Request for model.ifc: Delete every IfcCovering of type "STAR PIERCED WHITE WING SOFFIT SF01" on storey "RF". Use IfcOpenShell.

First a look at what the model holds.

```python
import ifcopenshell
import ifcopenshell.util.element

model = ifcopenshell.open("model.ifc")
print(model.schema)
storey = next(s for s in model.by_type("IfcBuildingStorey") if s.Name == "RF")
coverings = [e for e in ifcopenshell.util.element.get_decomposition(storey) if e.is_a("IfcCovering")]
seen = {}
for e in coverings:
    element_type = ifcopenshell.util.element.get_type(e)
    name = element_type.Name if element_type not in (None, e) else None
    seen[name] = seen.get(name, 0) + 1
for name, count in sorted(seen.items(), key=str):
    print(count, "x", name)
```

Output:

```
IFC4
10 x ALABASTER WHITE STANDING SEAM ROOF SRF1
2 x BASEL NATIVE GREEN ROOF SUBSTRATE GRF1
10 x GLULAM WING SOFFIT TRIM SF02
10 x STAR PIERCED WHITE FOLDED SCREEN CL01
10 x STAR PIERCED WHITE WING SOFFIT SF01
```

```python
import ifcopenshell
import ifcopenshell.api.root
import ifcopenshell.util.element

model = ifcopenshell.open("model.ifc")

storey = next(s for s in model.by_type("IfcBuildingStorey") if s.Name == "RF")
coverings = [e for e in ifcopenshell.util.element.get_decomposition(storey) if e.is_a("IfcCovering")]
targets = [e for e in coverings if (t := ifcopenshell.util.element.get_type(e)) not in (None, e) and t.Name == "STAR PIERCED WHITE WING SOFFIT SF01"]

for e in targets:
    ifcopenshell.api.root.remove_product(model, product=e)
print(len(targets), "removed")

model.write("model_v2.ifc")
```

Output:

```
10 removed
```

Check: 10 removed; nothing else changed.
